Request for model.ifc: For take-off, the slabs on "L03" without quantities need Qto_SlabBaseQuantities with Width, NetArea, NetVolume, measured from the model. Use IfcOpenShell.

First a look at what the model holds.

```python
import ifcopenshell
import ifcopenshell.util.element
import ifcopenshell.util.unit

model = ifcopenshell.open("model.ifc")
print(model.schema)
for unit_type in ("LENGTHUNIT", "AREAUNIT", "VOLUMEUNIT"):
    print(unit_type, ifcopenshell.util.unit.calculate_unit_scale(model, unit_type))
storey = next(s for s in model.by_type("IfcBuildingStorey") if s.Name == "L03")
slabs = [e for e in ifcopenshell.util.element.get_decomposition(storey) if e.is_a("IfcSlab")]
for e in sorted(slabs, key=lambda e: e.id()):
    print(e.id(), e.is_a(), e.Name, list(ifcopenshell.util.element.get_psets(e, qtos_only=True)), sep=" | ")
```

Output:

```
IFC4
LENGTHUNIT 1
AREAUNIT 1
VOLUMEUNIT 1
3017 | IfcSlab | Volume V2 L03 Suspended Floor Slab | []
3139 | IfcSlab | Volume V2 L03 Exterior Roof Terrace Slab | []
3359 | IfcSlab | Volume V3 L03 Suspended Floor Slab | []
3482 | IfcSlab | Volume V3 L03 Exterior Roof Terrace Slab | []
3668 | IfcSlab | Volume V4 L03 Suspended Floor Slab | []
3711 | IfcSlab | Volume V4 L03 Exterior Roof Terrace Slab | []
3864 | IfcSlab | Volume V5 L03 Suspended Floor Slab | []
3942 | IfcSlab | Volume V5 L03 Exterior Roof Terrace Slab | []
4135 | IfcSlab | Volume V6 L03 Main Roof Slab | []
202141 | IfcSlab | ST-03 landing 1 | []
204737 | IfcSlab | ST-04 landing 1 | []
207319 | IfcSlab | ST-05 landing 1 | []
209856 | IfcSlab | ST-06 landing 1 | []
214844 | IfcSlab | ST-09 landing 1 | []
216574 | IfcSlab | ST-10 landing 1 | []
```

```python
import ifcopenshell
import ifcopenshell.api.pset
import ifcopenshell.geom
import ifcopenshell.util.element
import ifcopenshell.util.shape
import ifcopenshell.util.unit

model = ifcopenshell.open("model.ifc")
unit_scale = ifcopenshell.util.unit.calculate_unit_scale(model)
area_scale = ifcopenshell.util.unit.calculate_unit_scale(model, "AREAUNIT")
volume_scale = ifcopenshell.util.unit.calculate_unit_scale(model, "VOLUMEUNIT")
settings = ifcopenshell.geom.settings()

storey = next(s for s in model.by_type("IfcBuildingStorey") if s.Name == "L03")
slabs = [e for e in ifcopenshell.util.element.get_decomposition(storey) if e.is_a("IfcSlab")]

for e in sorted(slabs, key=lambda e: e.id()):
    if ifcopenshell.util.element.get_psets(e, qtos_only=True, should_inherit=False):
        continue
    # Geometry comes back in metres, in the element's own axes.
    shape = ifcopenshell.geom.create_shape(settings, e)
    values = {
        "Width": ifcopenshell.util.shape.get_z(shape.geometry) / unit_scale,
        "NetArea": ifcopenshell.util.shape.get_footprint_area(shape.geometry) / area_scale,
        "NetVolume": ifcopenshell.util.shape.get_volume(shape.geometry) / volume_scale,
    }
    qto = ifcopenshell.api.pset.add_qto(model, product=e, name="Qto_SlabBaseQuantities")
    ifcopenshell.api.pset.edit_qto(model, qto=qto, properties=values)
    print(e.id(), {k: round(v, 3) for k, v in values.items()})

model.write("model_rev.ifc")
```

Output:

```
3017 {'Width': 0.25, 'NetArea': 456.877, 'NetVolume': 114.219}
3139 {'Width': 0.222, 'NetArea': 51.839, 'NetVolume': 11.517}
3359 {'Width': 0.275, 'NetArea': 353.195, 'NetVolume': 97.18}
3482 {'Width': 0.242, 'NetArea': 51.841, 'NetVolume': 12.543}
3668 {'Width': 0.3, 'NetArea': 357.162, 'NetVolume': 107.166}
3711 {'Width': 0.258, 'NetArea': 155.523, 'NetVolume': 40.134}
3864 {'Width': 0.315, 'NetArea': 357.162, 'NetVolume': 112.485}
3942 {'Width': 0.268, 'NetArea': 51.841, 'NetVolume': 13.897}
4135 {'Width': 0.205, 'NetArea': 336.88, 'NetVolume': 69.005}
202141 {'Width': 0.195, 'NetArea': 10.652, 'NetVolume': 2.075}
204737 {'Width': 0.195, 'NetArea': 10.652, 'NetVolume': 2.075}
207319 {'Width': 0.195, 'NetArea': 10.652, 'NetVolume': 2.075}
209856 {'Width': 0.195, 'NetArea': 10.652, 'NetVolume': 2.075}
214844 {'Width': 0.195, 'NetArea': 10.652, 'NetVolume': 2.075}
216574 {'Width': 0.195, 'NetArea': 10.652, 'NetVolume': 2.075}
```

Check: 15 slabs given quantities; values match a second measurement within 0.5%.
